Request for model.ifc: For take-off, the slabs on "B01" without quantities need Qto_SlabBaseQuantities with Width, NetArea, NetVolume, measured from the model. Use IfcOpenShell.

First a look at what the model holds.

```python
import ifcopenshell
import ifcopenshell.util.element
import ifcopenshell.util.unit

model = ifcopenshell.open("model.ifc")
print(model.schema)
for unit_type in ("LENGTHUNIT", "AREAUNIT", "VOLUMEUNIT"):
    print(unit_type, ifcopenshell.util.unit.calculate_unit_scale(model, unit_type))
storey = next(s for s in model.by_type("IfcBuildingStorey") if s.Name == "B01")
slabs = [e for e in ifcopenshell.util.element.get_decomposition(storey) if e.is_a("IfcSlab")]
for e in sorted(slabs, key=lambda e: e.id()):
    print(e.id(), e.is_a(), e.Name, list(ifcopenshell.util.element.get_psets(e, qtos_only=True)), sep=" | ")
```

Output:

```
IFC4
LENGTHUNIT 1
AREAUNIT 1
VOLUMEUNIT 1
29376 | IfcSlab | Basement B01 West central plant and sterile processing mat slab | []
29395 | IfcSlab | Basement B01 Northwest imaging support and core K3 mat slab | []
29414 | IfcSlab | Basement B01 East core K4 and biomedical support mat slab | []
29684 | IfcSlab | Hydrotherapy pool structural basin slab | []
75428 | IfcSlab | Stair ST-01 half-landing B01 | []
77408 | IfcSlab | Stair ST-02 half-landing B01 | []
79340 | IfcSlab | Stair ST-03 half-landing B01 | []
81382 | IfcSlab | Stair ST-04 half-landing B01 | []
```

```python
import ifcopenshell
import ifcopenshell.api.pset
import ifcopenshell.geom
import ifcopenshell.util.element
import ifcopenshell.util.shape
import ifcopenshell.util.unit

model = ifcopenshell.open("model.ifc")
unit_scale = ifcopenshell.util.unit.calculate_unit_scale(model)
area_scale = ifcopenshell.util.unit.calculate_unit_scale(model, "AREAUNIT")
volume_scale = ifcopenshell.util.unit.calculate_unit_scale(model, "VOLUMEUNIT")
settings = ifcopenshell.geom.settings()

storey = next(s for s in model.by_type("IfcBuildingStorey") if s.Name == "B01")
slabs = [e for e in ifcopenshell.util.element.get_decomposition(storey) if e.is_a("IfcSlab")]

for e in sorted(slabs, key=lambda e: e.id()):
    if ifcopenshell.util.element.get_psets(e, qtos_only=True, should_inherit=False):
        continue
    # Geometry comes back in metres, in the element's own axes.
    shape = ifcopenshell.geom.create_shape(settings, e)
    values = {
        "Width": ifcopenshell.util.shape.get_z(shape.geometry) / unit_scale,
        "NetArea": ifcopenshell.util.shape.get_footprint_area(shape.geometry) / area_scale,
        "NetVolume": ifcopenshell.util.shape.get_volume(shape.geometry) / volume_scale,
    }
    qto = ifcopenshell.api.pset.add_qto(model, product=e, name="Qto_SlabBaseQuantities")
    ifcopenshell.api.pset.edit_qto(model, qto=qto, properties=values)
    print(e.id(), {k: round(v, 3) for k, v in values.items()})

model.write("model_updated.ifc")
```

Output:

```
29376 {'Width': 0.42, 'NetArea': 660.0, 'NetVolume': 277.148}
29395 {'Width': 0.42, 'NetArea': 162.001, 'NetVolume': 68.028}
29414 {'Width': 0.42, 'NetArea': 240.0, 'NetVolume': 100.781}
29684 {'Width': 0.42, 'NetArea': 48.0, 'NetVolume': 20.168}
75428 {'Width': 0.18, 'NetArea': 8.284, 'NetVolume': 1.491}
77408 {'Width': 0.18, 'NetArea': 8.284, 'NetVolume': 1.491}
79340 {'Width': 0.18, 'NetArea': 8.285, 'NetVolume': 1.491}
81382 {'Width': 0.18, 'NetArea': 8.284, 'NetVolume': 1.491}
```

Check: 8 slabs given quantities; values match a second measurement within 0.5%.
